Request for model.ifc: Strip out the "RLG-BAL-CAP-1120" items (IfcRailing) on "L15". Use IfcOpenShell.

First a look at what the model holds.

```python
import ifcopenshell
import ifcopenshell.util.element

model = ifcopenshell.open("model.ifc")
print(model.schema)
storey = next(s for s in model.by_type("IfcBuildingStorey") if s.Name == "L15")
railings = [e for e in ifcopenshell.util.element.get_decomposition(storey) if e.is_a("IfcRailing")]
seen = {}
for e in railings:
    element_type = ifcopenshell.util.element.get_type(e)
    name = element_type.Name if element_type not in (None, e) else None
    seen[name] = seen.get(name, 0) + 1
for name, count in sorted(seen.items(), key=str):
    print(count, "x", name)
```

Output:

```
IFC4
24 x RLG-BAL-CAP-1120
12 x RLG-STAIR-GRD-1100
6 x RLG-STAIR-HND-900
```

```python
import ifcopenshell
import ifcopenshell.api.root
import ifcopenshell.util.element

model = ifcopenshell.open("model.ifc")

storey = next(s for s in model.by_type("IfcBuildingStorey") if s.Name == "L15")
railings = [e for e in ifcopenshell.util.element.get_decomposition(storey) if e.is_a("IfcRailing")]
targets = [e for e in railings if (t := ifcopenshell.util.element.get_type(e)) not in (None, e) and t.Name == "RLG-BAL-CAP-1120"]

for e in targets:
    ifcopenshell.api.root.remove_product(model, product=e)
print(len(targets), "removed")

model.write("model-out.ifc")
```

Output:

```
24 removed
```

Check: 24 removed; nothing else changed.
